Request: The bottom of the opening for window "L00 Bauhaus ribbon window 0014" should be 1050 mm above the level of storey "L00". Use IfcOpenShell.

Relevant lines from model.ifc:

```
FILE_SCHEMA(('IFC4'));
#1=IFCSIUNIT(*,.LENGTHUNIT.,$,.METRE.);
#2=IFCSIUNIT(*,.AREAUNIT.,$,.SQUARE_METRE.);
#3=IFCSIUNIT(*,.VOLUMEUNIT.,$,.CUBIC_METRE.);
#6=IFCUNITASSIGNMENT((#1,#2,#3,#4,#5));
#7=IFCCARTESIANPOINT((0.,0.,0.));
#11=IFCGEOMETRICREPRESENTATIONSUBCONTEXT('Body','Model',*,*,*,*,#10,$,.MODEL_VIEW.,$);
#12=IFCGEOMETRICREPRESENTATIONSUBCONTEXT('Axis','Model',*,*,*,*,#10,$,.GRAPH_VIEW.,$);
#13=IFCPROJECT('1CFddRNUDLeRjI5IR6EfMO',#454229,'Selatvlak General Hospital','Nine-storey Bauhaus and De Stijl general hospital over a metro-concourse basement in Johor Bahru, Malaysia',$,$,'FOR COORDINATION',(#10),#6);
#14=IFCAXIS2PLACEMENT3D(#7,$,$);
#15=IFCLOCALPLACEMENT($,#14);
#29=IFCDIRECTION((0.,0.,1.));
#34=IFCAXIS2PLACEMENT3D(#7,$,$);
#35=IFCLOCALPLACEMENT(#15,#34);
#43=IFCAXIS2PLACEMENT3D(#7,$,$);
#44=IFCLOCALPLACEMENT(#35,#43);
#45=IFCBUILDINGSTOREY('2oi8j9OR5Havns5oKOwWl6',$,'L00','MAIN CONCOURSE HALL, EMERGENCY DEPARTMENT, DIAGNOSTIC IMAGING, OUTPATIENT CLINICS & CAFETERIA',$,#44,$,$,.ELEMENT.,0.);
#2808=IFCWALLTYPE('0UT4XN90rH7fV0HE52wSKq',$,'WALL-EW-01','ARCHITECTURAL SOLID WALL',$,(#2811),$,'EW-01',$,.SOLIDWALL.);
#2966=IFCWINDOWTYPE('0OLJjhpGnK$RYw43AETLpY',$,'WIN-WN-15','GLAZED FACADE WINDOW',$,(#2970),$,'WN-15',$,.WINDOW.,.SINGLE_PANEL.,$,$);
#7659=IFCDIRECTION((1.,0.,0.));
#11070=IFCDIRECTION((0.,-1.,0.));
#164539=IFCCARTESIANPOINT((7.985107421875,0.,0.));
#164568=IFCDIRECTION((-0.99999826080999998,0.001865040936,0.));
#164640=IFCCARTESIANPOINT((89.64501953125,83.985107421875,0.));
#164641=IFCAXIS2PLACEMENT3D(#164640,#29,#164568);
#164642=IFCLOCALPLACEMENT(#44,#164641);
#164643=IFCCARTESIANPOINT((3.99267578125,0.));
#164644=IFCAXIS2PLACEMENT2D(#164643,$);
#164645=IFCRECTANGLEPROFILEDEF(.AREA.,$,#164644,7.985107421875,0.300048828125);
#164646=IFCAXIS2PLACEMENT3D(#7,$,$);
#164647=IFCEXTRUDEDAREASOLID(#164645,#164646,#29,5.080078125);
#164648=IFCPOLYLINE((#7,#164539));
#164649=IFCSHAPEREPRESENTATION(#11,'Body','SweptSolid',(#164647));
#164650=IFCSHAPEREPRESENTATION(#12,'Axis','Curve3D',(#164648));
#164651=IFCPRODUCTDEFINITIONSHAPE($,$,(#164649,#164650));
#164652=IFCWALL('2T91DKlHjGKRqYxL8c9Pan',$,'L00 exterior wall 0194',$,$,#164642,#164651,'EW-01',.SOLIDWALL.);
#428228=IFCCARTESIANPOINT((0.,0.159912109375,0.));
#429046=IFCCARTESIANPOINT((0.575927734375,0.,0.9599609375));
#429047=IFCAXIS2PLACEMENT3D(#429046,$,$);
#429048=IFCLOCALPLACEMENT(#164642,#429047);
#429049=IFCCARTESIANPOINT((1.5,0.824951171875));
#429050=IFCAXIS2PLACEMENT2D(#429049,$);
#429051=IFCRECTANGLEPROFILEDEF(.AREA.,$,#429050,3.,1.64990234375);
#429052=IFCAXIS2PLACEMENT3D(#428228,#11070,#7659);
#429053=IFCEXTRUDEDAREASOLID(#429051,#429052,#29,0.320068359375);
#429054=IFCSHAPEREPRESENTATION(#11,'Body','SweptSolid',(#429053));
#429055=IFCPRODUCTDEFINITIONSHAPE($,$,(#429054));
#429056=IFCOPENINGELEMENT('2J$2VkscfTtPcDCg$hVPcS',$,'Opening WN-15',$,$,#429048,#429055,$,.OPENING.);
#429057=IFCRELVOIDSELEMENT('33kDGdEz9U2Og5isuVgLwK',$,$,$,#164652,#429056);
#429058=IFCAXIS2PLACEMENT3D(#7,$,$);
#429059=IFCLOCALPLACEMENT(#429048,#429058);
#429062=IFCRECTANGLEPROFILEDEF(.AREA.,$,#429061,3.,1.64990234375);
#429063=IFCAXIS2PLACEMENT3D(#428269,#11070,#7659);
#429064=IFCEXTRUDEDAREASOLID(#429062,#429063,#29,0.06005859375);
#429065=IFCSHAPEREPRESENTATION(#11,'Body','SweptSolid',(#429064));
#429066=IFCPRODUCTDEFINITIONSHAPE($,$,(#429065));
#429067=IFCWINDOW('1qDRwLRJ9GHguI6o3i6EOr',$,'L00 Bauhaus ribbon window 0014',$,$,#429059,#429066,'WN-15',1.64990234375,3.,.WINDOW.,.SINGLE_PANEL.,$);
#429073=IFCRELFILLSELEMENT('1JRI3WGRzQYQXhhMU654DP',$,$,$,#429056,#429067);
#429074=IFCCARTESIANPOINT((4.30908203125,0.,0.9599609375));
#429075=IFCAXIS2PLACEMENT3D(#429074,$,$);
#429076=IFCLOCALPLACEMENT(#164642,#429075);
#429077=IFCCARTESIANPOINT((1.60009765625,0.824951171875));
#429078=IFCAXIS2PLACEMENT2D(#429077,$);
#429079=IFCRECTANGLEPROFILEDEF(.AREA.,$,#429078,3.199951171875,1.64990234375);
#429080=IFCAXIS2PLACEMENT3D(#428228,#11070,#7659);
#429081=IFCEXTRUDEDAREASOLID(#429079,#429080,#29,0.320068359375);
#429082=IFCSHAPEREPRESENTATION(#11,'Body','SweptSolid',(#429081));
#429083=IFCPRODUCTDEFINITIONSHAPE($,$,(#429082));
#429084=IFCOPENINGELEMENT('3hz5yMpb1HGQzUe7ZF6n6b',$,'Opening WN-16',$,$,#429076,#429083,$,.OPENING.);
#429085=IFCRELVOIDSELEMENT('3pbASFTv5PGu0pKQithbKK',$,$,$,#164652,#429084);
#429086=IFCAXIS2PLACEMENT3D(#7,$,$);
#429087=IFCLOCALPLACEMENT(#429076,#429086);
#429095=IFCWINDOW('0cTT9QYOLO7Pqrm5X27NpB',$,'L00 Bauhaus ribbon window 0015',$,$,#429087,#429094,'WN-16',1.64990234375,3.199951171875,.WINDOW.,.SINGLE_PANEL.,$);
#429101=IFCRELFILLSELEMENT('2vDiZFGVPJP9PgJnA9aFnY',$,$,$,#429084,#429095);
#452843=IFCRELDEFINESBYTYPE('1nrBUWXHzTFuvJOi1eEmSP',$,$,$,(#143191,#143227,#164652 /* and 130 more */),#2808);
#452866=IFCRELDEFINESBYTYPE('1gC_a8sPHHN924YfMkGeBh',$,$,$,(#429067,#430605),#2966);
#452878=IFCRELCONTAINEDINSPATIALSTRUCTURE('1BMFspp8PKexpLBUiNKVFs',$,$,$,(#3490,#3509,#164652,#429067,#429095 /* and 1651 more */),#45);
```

```python
import numpy as np
import ifcopenshell
import ifcopenshell.api.geometry
import ifcopenshell.geom
import ifcopenshell.util.element
import ifcopenshell.util.placement
import ifcopenshell.util.shape
import ifcopenshell.util.unit

model = ifcopenshell.open("model.ifc")
unit_scale = ifcopenshell.util.unit.calculate_unit_scale(model)

window = model.by_guid("1qDRwLRJ9GHguI6o3i6EOr")
opening = window.FillsVoids[0].RelatingOpeningElement
storey = ifcopenshell.util.element.get_container(window, ifc_class="IfcBuildingStorey")
level = ifcopenshell.util.placement.get_local_placement(storey.ObjectPlacement)[2, 3]

# The opening's origin need not be at the sill, so measure its lowest point.
shape = ifcopenshell.geom.create_shape(ifcopenshell.geom.settings(), opening)
bottom = ifcopenshell.util.shape.get_shape_bottom_elevation(shape, shape.geometry) / unit_scale
dz = level + 1.05 / unit_scale - bottom

shift = np.array([0.0, 0.0, dz])
# The window is placed relative to its opening, so it follows when the opening moves.
matrix = ifcopenshell.util.placement.get_local_placement(opening.ObjectPlacement)
matrix[:3, 3] += shift
ifcopenshell.api.geometry.edit_object_placement(
    model, product=opening, matrix=matrix, is_si=False, should_transform_children=True
)

print(f"moved by {dz * unit_scale:+.3f} m")

model.write("model_updated.ifc")
```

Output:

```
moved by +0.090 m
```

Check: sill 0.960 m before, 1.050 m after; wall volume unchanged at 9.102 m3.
